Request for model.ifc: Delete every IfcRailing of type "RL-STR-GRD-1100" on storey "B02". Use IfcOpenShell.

First a look at what the model holds.

```python
import ifcopenshell
import ifcopenshell.util.element

model = ifcopenshell.open("model.ifc")
print(model.schema)
storey = next(s for s in model.by_type("IfcBuildingStorey") if s.Name == "B02")
railings = [e for e in ifcopenshell.util.element.get_decomposition(storey) if e.is_a("IfcRailing")]
seen = {}
for e in railings:
    element_type = ifcopenshell.util.element.get_type(e)
    name = element_type.Name if element_type not in (None, e) else None
    seen[name] = seen.get(name, 0) + 1
for name, count in sorted(seen.items(), key=str):
    print(count, "x", name)
```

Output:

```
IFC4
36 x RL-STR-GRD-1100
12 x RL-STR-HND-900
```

```python
import ifcopenshell
import ifcopenshell.api.root
import ifcopenshell.util.element

model = ifcopenshell.open("model.ifc")

storey = next(s for s in model.by_type("IfcBuildingStorey") if s.Name == "B02")
railings = [e for e in ifcopenshell.util.element.get_decomposition(storey) if e.is_a("IfcRailing")]
targets = [e for e in railings if (t := ifcopenshell.util.element.get_type(e)) not in (None, e) and t.Name == "RL-STR-GRD-1100"]

for e in targets:
    ifcopenshell.api.root.remove_product(model, product=e)
print(len(targets), "removed")

model.write("model_updated.ifc")
```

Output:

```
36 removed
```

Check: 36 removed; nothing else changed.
